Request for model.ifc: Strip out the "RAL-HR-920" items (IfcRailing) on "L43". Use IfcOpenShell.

First a look at what the model holds.

```python
import ifcopenshell
import ifcopenshell.util.element

model = ifcopenshell.open("model.ifc")
print(model.schema)
storey = next(s for s in model.by_type("IfcBuildingStorey") if s.Name == "L43")
railings = [e for e in ifcopenshell.util.element.get_decomposition(storey) if e.is_a("IfcRailing")]
seen = {}
for e in railings:
    element_type = ifcopenshell.util.element.get_type(e)
    name = element_type.Name if element_type not in (None, e) else None
    seen[name] = seen.get(name, 0) + 1
for name, count in sorted(seen.items(), key=str):
    print(count, "x", name)
```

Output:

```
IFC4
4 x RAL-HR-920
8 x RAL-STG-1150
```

```python
import ifcopenshell
import ifcopenshell.api.root
import ifcopenshell.util.element

model = ifcopenshell.open("model.ifc")

storey = next(s for s in model.by_type("IfcBuildingStorey") if s.Name == "L43")
railings = [e for e in ifcopenshell.util.element.get_decomposition(storey) if e.is_a("IfcRailing")]
targets = [e for e in railings if (t := ifcopenshell.util.element.get_type(e)) not in (None, e) and t.Name == "RAL-HR-920"]

for e in targets:
    ifcopenshell.api.root.remove_product(model, product=e)
print(len(targets), "removed")

model.write("model_rev.ifc")
```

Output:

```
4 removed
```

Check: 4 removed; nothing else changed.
